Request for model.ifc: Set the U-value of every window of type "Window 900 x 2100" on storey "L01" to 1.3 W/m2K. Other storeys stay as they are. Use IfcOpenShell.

First a look at what the model holds.

```python
import ifcopenshell
import ifcopenshell.util.element

model = ifcopenshell.open("model.ifc")
print(model.schema)
storey = next(s for s in model.by_type("IfcBuildingStorey") if s.Name == "L01")
windows = [e for e in ifcopenshell.util.element.get_decomposition(storey) if e.is_a("IfcWindow")]
seen = {}
for e in windows:
    element_type = ifcopenshell.util.element.get_type(e)
    key = (element_type.Name if element_type != e and element_type else None, ifcopenshell.util.element.get_pset(e, "Pset_WindowCommon", "ThermalTransmittance"))
    seen[key] = seen.get(key, 0) + 1
for (name, value), count in sorted(seen.items(), key=str):
    print(count, "x", name, "|", value)
```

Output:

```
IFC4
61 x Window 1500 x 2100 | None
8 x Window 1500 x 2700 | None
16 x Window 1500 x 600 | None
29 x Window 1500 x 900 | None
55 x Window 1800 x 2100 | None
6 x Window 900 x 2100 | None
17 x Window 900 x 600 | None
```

```python
import ifcopenshell
import ifcopenshell.api.pset
import ifcopenshell.util.element

model = ifcopenshell.open("model.ifc")

storey = next(s for s in model.by_type("IfcBuildingStorey") if s.Name == "L01")
windows = [e for e in ifcopenshell.util.element.get_decomposition(storey) if e.is_a("IfcWindow")]

count = 0
for e in windows:
    element_type = ifcopenshell.util.element.get_type(e)
    if element_type in (None, e) or element_type.Name != "Window 900 x 2100":
        continue
    # add_pset returns the element's existing set when there is one.
    pset = ifcopenshell.api.pset.add_pset(model, product=e, name="Pset_WindowCommon")
    ifcopenshell.api.pset.edit_pset(model, pset=pset, properties={"ThermalTransmittance": 1.3})
    count += 1

print(count, "windows updated")

model.write("model_edited.ifc")
```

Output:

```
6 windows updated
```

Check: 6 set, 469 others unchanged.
